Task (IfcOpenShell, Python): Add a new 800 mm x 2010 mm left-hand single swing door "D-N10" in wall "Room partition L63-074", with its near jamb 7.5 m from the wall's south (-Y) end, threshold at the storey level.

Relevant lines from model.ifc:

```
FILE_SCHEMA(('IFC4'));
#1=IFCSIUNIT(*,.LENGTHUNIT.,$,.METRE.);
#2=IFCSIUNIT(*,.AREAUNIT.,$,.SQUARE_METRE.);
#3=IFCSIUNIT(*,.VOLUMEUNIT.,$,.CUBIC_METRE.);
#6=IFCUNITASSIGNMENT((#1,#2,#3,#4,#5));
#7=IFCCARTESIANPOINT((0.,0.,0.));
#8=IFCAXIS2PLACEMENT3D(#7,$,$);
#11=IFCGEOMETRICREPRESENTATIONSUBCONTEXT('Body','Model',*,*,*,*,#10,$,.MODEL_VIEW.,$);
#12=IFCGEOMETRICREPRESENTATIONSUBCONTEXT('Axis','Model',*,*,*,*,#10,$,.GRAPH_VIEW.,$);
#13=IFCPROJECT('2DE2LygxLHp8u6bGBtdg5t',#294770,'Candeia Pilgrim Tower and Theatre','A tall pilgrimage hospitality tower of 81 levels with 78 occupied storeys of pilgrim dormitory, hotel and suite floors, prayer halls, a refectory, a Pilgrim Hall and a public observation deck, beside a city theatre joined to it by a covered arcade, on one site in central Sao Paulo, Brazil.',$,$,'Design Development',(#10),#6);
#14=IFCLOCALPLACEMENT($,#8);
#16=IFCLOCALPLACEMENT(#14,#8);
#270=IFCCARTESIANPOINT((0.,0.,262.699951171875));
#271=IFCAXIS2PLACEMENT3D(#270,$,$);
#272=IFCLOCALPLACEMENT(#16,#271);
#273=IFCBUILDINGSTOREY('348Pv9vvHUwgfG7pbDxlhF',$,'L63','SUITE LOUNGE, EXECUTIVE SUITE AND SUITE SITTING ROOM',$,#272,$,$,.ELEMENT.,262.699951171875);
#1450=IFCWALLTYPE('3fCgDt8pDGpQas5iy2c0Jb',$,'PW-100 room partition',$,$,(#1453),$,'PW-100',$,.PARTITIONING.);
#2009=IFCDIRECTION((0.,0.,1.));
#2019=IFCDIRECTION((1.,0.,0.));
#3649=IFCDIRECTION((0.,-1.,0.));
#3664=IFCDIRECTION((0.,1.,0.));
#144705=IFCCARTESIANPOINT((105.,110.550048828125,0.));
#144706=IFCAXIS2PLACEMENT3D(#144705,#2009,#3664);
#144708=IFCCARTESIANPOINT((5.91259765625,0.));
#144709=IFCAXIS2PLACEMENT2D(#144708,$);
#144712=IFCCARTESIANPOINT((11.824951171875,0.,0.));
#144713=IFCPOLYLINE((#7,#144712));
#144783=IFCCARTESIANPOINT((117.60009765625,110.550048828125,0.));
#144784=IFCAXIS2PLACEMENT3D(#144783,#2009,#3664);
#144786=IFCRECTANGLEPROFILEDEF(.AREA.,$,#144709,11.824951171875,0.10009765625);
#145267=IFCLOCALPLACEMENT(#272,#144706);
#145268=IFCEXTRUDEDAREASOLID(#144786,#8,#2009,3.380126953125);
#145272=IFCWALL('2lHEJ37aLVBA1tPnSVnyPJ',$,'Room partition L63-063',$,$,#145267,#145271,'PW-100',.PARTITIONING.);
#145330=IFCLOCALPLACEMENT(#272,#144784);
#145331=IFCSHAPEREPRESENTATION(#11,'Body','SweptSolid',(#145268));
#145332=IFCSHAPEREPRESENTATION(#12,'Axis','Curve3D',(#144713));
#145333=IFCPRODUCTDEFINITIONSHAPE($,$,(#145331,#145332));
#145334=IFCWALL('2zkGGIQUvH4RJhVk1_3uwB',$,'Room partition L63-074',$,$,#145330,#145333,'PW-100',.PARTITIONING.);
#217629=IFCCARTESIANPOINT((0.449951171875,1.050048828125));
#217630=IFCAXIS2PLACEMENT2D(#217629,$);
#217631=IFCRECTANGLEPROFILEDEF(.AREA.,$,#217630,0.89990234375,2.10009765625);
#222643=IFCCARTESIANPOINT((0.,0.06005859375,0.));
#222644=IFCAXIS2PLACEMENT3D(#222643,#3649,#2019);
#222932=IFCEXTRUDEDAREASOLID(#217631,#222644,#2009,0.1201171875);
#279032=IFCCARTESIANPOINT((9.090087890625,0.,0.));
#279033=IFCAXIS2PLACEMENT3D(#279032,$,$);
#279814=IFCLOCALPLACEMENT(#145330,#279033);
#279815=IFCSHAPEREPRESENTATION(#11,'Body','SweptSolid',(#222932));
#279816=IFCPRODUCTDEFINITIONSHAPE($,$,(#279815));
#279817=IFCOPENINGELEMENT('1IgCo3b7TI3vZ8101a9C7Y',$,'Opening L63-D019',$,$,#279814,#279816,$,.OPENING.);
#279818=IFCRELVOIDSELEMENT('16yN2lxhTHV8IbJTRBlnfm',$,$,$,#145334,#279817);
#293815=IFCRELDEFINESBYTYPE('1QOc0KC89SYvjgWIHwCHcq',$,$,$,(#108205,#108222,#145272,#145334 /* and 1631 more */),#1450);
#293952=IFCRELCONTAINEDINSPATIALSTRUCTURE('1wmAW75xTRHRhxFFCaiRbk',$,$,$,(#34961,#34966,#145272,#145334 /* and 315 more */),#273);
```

```python
import numpy as np
import ifcopenshell
import ifcopenshell.api.feature
import ifcopenshell.api.geometry
import ifcopenshell.api.root
import ifcopenshell.api.spatial
import ifcopenshell.geom
import ifcopenshell.util.element
import ifcopenshell.util.placement
import ifcopenshell.util.representation
import ifcopenshell.util.shape
import ifcopenshell.util.unit

model = ifcopenshell.open("model.ifc")
unit_scale = ifcopenshell.util.unit.calculate_unit_scale(model)
settings = ifcopenshell.geom.settings()


def volume(element):
    """Net volume in cubic metres, openings subtracted."""
    shape = ifcopenshell.geom.create_shape(settings, element)
    return ifcopenshell.util.shape.get_volume(shape.geometry)


wall = model.by_id(145334)
storey = ifcopenshell.util.element.get_container(wall, ifc_class="IfcBuildingStorey")
context = ifcopenshell.util.representation.get_context(model, "Model", "Body", "MODEL_VIEW")
before = volume(wall)

width, height, from_end, sill = 0.8, 2.01, 7.5, 0.0  # metres

# The wall runs along its own X axis, and the end named is its -X end.
wall_shape = ifcopenshell.geom.create_shape(settings, wall)
x, y, z = ifcopenshell.util.shape.get_vertices(wall_shape.geometry).T
start = x.min() + from_end
face, thickness = float(y.min()), float(y.max() - y.min())
wall_matrix = ifcopenshell.util.placement.get_local_placement(wall.ObjectPlacement)
level = ifcopenshell.util.placement.get_local_placement(storey.ObjectPlacement)[2, 3]


def in_wall(x, y):
    """Placement at x, y metres in the wall's axes, at sill height."""
    matrix = wall_matrix.copy()
    matrix[:, 3] = wall_matrix @ np.array([x / unit_scale, y / unit_scale, 0.0, 1.0])
    matrix[2, 3] = level + sill / unit_scale
    return matrix


# Opening: a box that overshoots both wall faces by 50 mm.
opening = ifcopenshell.api.root.create_entity(model, ifc_class="IfcOpeningElement", predefined_type="OPENING")
box = ifcopenshell.api.geometry.add_wall_representation(
    model, context=context, length=width, height=height, thickness=thickness + 0.1
)
ifcopenshell.api.geometry.assign_representation(model, product=opening, representation=box)
ifcopenshell.api.geometry.edit_object_placement(model, product=opening, matrix=in_wall(start, face - 0.05), is_si=False)
ifcopenshell.api.feature.add_feature(model, feature=opening, element=wall)

door = ifcopenshell.api.root.create_entity(model, ifc_class="IfcDoor", name="D-N10", predefined_type="DOOR")
door.OverallWidth, door.OverallHeight = width / unit_scale, height / unit_scale
door.OperationType = "SINGLE_SWING_LEFT"
body = ifcopenshell.api.geometry.add_door_representation(
    model,
    context=context,
    overall_width=door.OverallWidth,
    overall_height=door.OverallHeight,
    operation_type="SINGLE_SWING_LEFT",
    lining_properties={"LiningDepth": thickness / unit_scale, "ThresholdDepth": thickness / unit_scale},
)
ifcopenshell.api.geometry.assign_representation(model, product=door, representation=body)
ifcopenshell.api.spatial.assign_container(model, products=[door], relating_structure=storey)
ifcopenshell.api.feature.add_filling(model, opening=opening, element=door)

# The lining spans the wall, so the door starts at the wall face.
ifcopenshell.api.geometry.edit_object_placement(model, product=door, matrix=in_wall(start, face), is_si=False)

after = volume(wall)

print(f"wall volume {before:.3f} -> {after:.3f} m3")

model.write("model-out.ifc")
```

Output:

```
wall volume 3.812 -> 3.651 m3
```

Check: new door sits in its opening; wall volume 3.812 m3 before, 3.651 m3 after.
